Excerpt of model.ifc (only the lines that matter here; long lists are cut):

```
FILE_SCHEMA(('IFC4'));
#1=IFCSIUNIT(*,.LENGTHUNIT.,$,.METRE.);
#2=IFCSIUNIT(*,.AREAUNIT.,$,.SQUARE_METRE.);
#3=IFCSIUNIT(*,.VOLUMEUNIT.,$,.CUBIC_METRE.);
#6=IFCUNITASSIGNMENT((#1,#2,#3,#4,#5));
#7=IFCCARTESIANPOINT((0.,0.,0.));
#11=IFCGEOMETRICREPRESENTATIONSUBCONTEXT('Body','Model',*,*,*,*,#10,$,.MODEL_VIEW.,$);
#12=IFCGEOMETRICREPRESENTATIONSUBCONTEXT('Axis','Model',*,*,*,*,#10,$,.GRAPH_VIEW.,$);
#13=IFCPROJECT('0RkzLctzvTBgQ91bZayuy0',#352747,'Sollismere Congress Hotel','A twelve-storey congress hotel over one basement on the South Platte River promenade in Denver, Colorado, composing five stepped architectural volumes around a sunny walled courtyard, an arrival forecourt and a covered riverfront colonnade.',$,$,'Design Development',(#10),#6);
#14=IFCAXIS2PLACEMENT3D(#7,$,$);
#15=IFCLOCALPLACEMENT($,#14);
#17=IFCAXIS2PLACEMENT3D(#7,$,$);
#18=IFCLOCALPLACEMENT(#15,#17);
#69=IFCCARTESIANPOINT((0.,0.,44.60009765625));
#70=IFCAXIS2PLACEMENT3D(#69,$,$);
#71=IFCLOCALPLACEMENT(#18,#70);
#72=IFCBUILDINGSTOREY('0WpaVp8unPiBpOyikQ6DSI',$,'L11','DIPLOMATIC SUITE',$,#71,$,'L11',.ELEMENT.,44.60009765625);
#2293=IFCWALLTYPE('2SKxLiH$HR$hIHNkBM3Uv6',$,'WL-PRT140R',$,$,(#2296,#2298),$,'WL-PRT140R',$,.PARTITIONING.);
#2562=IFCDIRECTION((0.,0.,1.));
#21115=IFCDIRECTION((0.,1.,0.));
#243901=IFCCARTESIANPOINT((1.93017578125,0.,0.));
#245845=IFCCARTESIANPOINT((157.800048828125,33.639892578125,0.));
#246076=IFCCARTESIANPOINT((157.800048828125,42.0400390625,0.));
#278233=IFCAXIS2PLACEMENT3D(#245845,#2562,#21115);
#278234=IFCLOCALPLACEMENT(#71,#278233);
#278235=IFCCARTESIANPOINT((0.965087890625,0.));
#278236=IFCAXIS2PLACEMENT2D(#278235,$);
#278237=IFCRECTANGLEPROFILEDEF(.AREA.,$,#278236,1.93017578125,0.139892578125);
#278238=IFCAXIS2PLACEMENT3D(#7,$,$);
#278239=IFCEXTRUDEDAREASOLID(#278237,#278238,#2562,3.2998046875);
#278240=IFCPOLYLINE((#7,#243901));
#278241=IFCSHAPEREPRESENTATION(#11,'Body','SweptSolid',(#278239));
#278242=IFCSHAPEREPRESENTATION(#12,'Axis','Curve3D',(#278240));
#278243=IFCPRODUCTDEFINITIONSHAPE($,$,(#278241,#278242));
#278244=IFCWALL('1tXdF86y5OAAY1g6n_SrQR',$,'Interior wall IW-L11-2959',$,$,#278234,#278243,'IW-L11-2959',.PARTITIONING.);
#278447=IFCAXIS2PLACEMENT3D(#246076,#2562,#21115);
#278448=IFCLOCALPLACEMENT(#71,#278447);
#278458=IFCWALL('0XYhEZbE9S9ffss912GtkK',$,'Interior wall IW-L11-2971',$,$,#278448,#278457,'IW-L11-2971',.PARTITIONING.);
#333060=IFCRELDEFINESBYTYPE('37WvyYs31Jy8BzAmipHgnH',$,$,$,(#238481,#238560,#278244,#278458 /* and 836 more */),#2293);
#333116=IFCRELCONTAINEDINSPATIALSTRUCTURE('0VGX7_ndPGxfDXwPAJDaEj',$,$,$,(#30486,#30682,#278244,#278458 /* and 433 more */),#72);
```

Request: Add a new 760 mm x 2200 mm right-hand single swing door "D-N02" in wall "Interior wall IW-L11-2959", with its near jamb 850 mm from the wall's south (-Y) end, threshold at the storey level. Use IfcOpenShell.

```python
import numpy as np
import ifcopenshell
import ifcopenshell.api.feature
import ifcopenshell.api.geometry
import ifcopenshell.api.root
import ifcopenshell.api.spatial
import ifcopenshell.geom
import ifcopenshell.util.element
import ifcopenshell.util.placement
import ifcopenshell.util.representation
import ifcopenshell.util.shape
import ifcopenshell.util.unit

model = ifcopenshell.open("model.ifc")
unit_scale = ifcopenshell.util.unit.calculate_unit_scale(model)
settings = ifcopenshell.geom.settings()


def volume(element):
    """Net volume in cubic metres, openings subtracted."""
    shape = ifcopenshell.geom.create_shape(settings, element)
    return ifcopenshell.util.shape.get_volume(shape.geometry)


wall = model.by_guid("1tXdF86y5OAAY1g6n_SrQR")
storey = ifcopenshell.util.element.get_container(wall, ifc_class="IfcBuildingStorey")
context = ifcopenshell.util.representation.get_context(model, "Model", "Body", "MODEL_VIEW")
before = volume(wall)

width, height, from_end, sill = 0.76, 2.2, 0.85, 0.0  # metres

# The wall runs along its own X axis, and the end named is its -X end.
wall_shape = ifcopenshell.geom.create_shape(settings, wall)
x, y, z = ifcopenshell.util.shape.get_vertices(wall_shape.geometry).T
start = x.min() + from_end
face, thickness = float(y.min()), float(y.max() - y.min())
wall_matrix = ifcopenshell.util.placement.get_local_placement(wall.ObjectPlacement)
level = ifcopenshell.util.placement.get_local_placement(storey.ObjectPlacement)[2, 3]


def in_wall(x, y):
    """Placement at x, y metres in the wall's axes, at sill height."""
    matrix = wall_matrix.copy()
    matrix[:, 3] = wall_matrix @ np.array([x / unit_scale, y / unit_scale, 0.0, 1.0])
    matrix[2, 3] = level + sill / unit_scale
    return matrix


# Opening: a box that overshoots both wall faces by 50 mm.
opening = ifcopenshell.api.root.create_entity(model, ifc_class="IfcOpeningElement", predefined_type="OPENING")
box = ifcopenshell.api.geometry.add_wall_representation(
    model, context=context, length=width, height=height, thickness=thickness + 0.1
)
ifcopenshell.api.geometry.assign_representation(model, product=opening, representation=box)
ifcopenshell.api.geometry.edit_object_placement(model, product=opening, matrix=in_wall(start, face - 0.05), is_si=False)
ifcopenshell.api.feature.add_feature(model, feature=opening, element=wall)

door = ifcopenshell.api.root.create_entity(model, ifc_class="IfcDoor", name="D-N02", predefined_type="DOOR")
door.OverallWidth, door.OverallHeight = width / unit_scale, height / unit_scale
door.OperationType = "SINGLE_SWING_RIGHT"
body = ifcopenshell.api.geometry.add_door_representation(
    model,
    context=context,
    overall_width=door.OverallWidth,
    overall_height=door.OverallHeight,
    operation_type="SINGLE_SWING_RIGHT",
    lining_properties={"LiningDepth": thickness / unit_scale, "ThresholdDepth": thickness / unit_scale},
)
ifcopenshell.api.geometry.assign_representation(model, product=door, representation=body)
ifcopenshell.api.spatial.assign_container(model, products=[door], relating_structure=storey)
ifcopenshell.api.feature.add_filling(model, opening=opening, element=door)

# The lining spans the wall, so the door starts at the wall face.
ifcopenshell.api.geometry.edit_object_placement(model, product=door, matrix=in_wall(start, face), is_si=False)

after = volume(wall)

print(f"wall volume {before:.3f} -> {after:.3f} m3")

model.write("model-out.ifc")
```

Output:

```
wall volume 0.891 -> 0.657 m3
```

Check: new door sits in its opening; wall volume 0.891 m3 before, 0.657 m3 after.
